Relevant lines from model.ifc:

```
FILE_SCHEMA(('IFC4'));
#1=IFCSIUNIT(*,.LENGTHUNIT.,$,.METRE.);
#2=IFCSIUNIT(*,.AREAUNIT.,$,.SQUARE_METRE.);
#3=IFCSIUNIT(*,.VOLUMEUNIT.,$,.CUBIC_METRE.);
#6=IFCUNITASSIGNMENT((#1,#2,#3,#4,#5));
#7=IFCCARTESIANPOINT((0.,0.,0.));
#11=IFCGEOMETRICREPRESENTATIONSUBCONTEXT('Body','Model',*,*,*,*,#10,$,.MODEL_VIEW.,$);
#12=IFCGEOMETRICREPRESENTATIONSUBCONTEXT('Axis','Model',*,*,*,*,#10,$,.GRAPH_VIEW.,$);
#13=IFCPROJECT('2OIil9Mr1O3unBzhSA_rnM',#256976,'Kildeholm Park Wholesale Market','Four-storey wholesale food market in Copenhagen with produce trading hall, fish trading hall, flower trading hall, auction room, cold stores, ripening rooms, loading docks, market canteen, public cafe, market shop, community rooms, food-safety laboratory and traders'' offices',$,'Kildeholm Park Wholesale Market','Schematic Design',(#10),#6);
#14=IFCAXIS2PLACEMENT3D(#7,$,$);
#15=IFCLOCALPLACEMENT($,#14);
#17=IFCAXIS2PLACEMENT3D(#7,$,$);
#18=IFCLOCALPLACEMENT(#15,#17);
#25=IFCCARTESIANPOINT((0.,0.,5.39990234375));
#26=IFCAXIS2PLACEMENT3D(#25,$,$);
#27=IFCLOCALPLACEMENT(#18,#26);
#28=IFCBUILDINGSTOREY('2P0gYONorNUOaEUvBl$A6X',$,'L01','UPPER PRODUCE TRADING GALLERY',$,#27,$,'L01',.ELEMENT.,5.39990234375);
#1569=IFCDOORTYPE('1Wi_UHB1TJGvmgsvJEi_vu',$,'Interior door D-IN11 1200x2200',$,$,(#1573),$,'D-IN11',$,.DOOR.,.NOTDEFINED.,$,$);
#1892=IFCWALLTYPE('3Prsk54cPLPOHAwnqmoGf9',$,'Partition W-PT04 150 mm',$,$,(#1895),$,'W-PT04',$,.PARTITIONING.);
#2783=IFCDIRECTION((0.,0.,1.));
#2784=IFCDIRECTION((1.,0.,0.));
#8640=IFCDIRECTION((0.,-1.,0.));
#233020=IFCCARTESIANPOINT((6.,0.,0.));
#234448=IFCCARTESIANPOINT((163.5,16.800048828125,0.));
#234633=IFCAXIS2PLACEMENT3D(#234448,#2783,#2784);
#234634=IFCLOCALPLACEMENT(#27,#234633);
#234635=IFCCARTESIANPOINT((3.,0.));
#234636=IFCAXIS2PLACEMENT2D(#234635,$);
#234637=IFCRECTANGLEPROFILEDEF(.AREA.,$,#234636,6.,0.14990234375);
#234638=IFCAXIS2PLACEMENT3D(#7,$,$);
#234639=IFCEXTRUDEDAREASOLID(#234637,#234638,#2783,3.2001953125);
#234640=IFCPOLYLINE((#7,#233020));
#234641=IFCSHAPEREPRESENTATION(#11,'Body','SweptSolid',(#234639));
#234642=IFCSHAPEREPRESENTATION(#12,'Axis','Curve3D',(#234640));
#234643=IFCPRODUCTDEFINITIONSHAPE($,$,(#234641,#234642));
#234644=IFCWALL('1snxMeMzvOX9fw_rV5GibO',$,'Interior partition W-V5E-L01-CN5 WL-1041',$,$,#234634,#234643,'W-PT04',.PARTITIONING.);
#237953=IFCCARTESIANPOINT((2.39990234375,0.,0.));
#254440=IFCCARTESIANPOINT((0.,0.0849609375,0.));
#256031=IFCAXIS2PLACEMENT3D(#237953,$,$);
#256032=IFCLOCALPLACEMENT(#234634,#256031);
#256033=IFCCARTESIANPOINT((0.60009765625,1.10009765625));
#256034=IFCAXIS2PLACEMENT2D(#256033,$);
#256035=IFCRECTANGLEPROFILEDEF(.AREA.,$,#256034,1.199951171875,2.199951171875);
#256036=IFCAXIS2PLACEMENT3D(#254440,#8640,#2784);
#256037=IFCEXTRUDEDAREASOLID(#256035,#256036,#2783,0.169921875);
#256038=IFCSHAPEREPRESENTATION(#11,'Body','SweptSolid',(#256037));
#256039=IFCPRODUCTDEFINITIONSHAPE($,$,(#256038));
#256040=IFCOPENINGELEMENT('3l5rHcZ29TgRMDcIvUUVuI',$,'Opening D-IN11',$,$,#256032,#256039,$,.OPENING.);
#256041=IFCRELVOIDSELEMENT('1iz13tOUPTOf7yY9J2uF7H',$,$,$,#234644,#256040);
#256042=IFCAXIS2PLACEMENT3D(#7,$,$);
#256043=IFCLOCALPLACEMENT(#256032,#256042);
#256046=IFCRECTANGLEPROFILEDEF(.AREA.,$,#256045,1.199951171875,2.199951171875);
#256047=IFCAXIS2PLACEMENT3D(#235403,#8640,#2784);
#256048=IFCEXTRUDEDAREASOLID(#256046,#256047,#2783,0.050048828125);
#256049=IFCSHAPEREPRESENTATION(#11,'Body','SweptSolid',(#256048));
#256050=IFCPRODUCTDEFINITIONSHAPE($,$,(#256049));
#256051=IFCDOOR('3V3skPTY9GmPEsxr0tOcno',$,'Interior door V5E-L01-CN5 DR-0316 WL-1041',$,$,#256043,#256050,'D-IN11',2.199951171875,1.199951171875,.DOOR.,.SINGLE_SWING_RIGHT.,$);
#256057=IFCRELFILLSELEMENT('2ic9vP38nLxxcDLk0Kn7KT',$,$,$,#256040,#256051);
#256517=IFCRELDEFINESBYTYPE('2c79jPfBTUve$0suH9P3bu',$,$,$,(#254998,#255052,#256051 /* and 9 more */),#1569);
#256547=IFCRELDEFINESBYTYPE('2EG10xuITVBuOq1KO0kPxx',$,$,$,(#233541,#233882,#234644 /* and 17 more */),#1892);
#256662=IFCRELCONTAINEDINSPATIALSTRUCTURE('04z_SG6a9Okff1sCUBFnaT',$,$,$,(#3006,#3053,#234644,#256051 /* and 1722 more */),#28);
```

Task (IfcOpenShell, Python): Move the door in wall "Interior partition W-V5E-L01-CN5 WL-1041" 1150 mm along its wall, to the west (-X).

```python
import ifcopenshell
import ifcopenshell.api.geometry
import ifcopenshell.util.placement
import ifcopenshell.util.unit

model = ifcopenshell.open("model.ifc")
unit_scale = ifcopenshell.util.unit.calculate_unit_scale(model)

door = model.by_id(256051)
opening = door.FillsVoids[0].RelatingOpeningElement
wall = opening.VoidsElements[0].RelatingBuildingElement

wall_matrix = ifcopenshell.util.placement.get_local_placement(wall.ObjectPlacement)
shift = wall_matrix[:3, 0] * -1.15 / unit_scale
before = ifcopenshell.util.placement.get_local_placement(door.ObjectPlacement)[:3, 3].copy()

# The door is placed relative to its opening, so it follows when the opening moves.
matrix = ifcopenshell.util.placement.get_local_placement(opening.ObjectPlacement)
matrix[:3, 3] += shift
ifcopenshell.api.geometry.edit_object_placement(
    model, product=opening, matrix=matrix, is_si=False, should_transform_children=True
)

after = ifcopenshell.util.placement.get_local_placement(door.ObjectPlacement)[:3, 3]
print("door moved by", (after - before).round(3) + 0.0)

model.write("model_rev.ifc")
```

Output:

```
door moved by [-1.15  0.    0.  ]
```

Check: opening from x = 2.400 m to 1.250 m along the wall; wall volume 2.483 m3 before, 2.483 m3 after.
